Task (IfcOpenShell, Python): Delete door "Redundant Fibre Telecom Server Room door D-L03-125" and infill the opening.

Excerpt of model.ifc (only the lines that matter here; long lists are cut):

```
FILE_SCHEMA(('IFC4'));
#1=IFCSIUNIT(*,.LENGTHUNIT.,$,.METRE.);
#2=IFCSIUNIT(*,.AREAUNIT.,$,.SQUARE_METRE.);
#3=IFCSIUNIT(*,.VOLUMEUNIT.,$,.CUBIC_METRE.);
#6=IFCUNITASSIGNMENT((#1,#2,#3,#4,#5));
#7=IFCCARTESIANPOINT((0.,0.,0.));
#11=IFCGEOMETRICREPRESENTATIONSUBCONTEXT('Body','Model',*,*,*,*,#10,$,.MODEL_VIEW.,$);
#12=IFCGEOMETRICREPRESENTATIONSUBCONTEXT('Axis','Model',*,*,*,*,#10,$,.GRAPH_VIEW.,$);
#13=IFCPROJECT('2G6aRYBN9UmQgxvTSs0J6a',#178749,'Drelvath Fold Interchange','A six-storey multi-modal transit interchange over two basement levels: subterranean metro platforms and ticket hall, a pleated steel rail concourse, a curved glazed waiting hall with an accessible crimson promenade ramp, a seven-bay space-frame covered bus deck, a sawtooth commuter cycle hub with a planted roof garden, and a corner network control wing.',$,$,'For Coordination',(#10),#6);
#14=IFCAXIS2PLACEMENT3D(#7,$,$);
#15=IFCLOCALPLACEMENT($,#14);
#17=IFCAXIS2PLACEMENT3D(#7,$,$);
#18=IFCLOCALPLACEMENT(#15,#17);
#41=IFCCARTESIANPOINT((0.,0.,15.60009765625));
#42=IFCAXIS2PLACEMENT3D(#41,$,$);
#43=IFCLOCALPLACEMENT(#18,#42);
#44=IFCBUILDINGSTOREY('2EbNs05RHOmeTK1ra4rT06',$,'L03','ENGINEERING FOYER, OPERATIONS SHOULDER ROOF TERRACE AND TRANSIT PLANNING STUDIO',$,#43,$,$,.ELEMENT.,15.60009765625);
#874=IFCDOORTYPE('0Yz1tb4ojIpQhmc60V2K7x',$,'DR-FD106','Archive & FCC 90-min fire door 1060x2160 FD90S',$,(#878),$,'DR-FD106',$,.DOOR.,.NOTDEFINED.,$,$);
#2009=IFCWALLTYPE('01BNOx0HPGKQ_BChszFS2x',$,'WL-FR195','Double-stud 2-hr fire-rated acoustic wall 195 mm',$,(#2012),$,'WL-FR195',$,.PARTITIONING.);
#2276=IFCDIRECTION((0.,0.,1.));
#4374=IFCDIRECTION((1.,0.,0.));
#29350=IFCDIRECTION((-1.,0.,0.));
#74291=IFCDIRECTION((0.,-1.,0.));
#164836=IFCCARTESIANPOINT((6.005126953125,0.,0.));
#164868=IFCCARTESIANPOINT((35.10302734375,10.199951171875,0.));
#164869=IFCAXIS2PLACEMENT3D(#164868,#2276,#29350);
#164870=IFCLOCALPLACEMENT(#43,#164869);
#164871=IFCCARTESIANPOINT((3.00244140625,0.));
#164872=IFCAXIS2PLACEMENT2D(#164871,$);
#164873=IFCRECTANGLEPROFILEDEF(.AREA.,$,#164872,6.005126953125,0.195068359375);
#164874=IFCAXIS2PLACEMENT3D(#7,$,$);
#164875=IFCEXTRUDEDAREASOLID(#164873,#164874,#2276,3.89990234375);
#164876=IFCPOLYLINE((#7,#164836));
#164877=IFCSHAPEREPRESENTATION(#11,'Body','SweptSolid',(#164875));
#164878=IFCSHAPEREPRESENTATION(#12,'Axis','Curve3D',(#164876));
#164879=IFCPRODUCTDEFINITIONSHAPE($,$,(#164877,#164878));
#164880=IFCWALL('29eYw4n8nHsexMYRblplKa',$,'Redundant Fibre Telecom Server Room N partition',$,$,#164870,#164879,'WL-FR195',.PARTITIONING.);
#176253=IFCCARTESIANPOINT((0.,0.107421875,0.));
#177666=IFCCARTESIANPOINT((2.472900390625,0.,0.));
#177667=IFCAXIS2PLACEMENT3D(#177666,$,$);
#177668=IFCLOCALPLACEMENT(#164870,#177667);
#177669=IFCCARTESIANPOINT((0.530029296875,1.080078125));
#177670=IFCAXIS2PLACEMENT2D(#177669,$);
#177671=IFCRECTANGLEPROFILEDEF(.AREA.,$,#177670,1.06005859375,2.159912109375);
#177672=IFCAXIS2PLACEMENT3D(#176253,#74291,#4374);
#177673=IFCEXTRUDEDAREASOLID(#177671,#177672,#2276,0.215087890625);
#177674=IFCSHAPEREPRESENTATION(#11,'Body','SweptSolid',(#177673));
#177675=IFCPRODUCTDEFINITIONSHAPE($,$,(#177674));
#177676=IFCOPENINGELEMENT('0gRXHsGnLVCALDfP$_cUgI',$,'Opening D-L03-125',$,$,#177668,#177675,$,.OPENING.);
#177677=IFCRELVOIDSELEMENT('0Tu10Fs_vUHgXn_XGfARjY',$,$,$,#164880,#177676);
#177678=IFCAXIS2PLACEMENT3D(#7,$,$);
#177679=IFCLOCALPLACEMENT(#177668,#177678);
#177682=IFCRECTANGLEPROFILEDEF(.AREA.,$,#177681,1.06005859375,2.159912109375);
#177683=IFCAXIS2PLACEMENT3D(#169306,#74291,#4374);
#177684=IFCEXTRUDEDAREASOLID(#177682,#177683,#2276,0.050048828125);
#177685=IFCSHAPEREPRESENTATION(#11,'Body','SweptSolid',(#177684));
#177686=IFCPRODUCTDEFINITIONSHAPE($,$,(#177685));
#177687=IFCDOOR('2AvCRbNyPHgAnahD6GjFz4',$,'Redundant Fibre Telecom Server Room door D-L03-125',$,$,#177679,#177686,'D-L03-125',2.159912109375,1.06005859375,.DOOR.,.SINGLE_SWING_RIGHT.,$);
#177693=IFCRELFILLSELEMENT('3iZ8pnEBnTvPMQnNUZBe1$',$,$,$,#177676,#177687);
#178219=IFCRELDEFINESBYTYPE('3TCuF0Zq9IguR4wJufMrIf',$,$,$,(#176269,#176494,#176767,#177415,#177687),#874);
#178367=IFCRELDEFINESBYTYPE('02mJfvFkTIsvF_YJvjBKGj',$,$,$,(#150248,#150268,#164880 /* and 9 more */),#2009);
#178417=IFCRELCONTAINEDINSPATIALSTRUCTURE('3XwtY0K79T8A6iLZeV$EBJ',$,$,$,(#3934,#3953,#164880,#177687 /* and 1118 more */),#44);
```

```python
import ifcopenshell
import ifcopenshell.api.feature
import ifcopenshell.api.root
import ifcopenshell.geom
import ifcopenshell.util.shape

model = ifcopenshell.open("model.ifc")
settings = ifcopenshell.geom.settings()


def volume(element):
    """Net volume in cubic metres, openings subtracted."""
    shape = ifcopenshell.geom.create_shape(settings, element)
    return ifcopenshell.util.shape.get_volume(shape.geometry)


door = model.by_id(177687)
opening = door.FillsVoids[0].RelatingOpeningElement
wall = opening.VoidsElements[0].RelatingBuildingElement
before = volume(wall)

ifcopenshell.api.root.remove_product(model, product=door)
ifcopenshell.api.feature.remove_feature(model, feature=opening)

after = volume(wall)

print(f"wall volume {before:.3f} -> {after:.3f} m3")

model.write("model_rev.ifc")
```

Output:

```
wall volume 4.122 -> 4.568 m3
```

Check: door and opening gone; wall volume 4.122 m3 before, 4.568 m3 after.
